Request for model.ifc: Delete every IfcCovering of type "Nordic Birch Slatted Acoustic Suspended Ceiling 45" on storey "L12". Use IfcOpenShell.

First a look at what the model holds.

```python
import ifcopenshell
import ifcopenshell.util.element

model = ifcopenshell.open("model.ifc")
print(model.schema)
storey = next(s for s in model.by_type("IfcBuildingStorey") if s.Name == "L12")
coverings = [e for e in ifcopenshell.util.element.get_decomposition(storey) if e.is_a("IfcCovering")]
seen = {}
for e in coverings:
    element_type = ifcopenshell.util.element.get_type(e)
    name = element_type.Name if element_type not in (None, e) else None
    seen[name] = seen.get(name, 0) + 1
for name, count in sorted(seen.items(), key=str):
    print(count, "x", name)
```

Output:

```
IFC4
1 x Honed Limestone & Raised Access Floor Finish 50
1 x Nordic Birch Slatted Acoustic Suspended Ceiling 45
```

```python
import ifcopenshell
import ifcopenshell.api.root
import ifcopenshell.util.element

model = ifcopenshell.open("model.ifc")

storey = next(s for s in model.by_type("IfcBuildingStorey") if s.Name == "L12")
coverings = [e for e in ifcopenshell.util.element.get_decomposition(storey) if e.is_a("IfcCovering")]
targets = [e for e in coverings if (t := ifcopenshell.util.element.get_type(e)) not in (None, e) and t.Name == "Nordic Birch Slatted Acoustic Suspended Ceiling 45"]

for e in targets:
    ifcopenshell.api.root.remove_product(model, product=e)
print(len(targets), "removed")

model.write("model_rev.ifc")
```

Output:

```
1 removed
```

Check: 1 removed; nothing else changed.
